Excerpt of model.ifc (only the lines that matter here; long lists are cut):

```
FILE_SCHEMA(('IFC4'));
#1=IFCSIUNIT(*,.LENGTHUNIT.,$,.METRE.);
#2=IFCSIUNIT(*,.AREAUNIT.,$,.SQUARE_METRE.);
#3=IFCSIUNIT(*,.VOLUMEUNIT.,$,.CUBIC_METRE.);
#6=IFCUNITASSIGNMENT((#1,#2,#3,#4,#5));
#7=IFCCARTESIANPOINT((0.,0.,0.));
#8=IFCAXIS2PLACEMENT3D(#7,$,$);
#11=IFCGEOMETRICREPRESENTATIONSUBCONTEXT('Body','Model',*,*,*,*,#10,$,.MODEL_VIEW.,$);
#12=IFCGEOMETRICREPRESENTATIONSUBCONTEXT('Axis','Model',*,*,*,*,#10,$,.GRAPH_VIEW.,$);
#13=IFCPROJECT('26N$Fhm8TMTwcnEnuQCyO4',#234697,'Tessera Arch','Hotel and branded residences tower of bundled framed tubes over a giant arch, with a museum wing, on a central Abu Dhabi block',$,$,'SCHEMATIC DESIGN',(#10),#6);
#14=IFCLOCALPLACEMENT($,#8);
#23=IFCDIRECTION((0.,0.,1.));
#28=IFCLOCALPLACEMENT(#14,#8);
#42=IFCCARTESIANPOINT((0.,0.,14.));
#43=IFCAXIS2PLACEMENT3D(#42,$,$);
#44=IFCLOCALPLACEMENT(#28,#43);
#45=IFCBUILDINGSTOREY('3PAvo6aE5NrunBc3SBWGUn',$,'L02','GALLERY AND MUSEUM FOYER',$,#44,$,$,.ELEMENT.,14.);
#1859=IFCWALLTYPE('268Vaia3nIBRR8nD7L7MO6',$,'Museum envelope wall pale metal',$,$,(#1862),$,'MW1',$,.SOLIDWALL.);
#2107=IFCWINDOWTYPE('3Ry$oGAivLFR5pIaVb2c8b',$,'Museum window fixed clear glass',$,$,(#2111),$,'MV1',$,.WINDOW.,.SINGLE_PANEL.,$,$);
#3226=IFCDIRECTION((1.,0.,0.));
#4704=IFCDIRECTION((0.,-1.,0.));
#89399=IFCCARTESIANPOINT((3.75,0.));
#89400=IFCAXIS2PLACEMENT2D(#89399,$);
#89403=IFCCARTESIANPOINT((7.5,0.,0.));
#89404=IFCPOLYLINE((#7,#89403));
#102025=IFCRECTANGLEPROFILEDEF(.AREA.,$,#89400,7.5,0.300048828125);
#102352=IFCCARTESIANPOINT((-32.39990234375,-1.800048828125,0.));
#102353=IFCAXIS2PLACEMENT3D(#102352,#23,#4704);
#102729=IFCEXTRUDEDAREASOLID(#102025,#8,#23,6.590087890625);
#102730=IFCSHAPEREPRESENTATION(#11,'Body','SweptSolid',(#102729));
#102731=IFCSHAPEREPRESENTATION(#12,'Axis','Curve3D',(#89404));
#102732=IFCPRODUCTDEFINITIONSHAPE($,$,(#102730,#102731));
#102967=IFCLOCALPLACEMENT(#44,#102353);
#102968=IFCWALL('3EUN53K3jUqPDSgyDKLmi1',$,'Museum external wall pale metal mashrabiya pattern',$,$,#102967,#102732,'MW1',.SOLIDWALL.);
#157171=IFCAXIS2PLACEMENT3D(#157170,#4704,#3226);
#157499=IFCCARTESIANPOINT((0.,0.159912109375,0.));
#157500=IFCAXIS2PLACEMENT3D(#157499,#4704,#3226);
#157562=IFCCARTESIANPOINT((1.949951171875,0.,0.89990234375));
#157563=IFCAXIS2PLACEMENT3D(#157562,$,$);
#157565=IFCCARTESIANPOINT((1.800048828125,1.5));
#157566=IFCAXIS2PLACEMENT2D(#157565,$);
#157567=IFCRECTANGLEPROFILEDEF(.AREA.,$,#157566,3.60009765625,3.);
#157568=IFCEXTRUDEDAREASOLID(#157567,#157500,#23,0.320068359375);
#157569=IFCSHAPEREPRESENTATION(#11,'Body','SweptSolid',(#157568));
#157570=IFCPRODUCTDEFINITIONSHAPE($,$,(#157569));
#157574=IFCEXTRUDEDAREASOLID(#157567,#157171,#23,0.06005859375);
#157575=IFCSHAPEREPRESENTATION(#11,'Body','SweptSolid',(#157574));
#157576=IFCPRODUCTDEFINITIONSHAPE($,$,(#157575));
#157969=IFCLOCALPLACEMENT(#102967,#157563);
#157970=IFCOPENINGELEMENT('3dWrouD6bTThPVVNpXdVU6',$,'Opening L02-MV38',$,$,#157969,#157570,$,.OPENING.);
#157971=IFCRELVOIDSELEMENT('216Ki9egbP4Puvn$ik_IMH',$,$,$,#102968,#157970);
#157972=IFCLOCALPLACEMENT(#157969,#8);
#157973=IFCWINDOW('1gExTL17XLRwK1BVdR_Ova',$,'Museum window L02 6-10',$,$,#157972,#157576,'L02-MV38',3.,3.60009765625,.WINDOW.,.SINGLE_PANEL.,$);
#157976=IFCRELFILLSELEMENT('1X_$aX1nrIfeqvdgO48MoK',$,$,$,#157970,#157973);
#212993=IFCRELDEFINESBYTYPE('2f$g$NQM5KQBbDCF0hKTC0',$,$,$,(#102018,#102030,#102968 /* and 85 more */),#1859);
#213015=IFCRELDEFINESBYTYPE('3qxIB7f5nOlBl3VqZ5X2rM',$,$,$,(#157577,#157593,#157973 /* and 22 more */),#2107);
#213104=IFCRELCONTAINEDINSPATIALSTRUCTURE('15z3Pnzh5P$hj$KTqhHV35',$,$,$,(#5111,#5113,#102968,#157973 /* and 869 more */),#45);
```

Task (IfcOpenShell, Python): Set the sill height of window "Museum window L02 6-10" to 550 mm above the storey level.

```python
import numpy as np
import ifcopenshell
import ifcopenshell.api.geometry
import ifcopenshell.geom
import ifcopenshell.util.element
import ifcopenshell.util.placement
import ifcopenshell.util.shape
import ifcopenshell.util.unit

model = ifcopenshell.open("model.ifc")
unit_scale = ifcopenshell.util.unit.calculate_unit_scale(model)

window = model.by_guid("1gExTL17XLRwK1BVdR_Ova")
opening = window.FillsVoids[0].RelatingOpeningElement
storey = ifcopenshell.util.element.get_container(window, ifc_class="IfcBuildingStorey")
level = ifcopenshell.util.placement.get_local_placement(storey.ObjectPlacement)[2, 3]

# The opening's origin need not be at the sill, so measure its lowest point.
shape = ifcopenshell.geom.create_shape(ifcopenshell.geom.settings(), opening)
bottom = ifcopenshell.util.shape.get_shape_bottom_elevation(shape, shape.geometry) / unit_scale
dz = level + 0.55 - bottom

shift = np.array([0.0, 0.0, dz])
# The window is placed relative to its opening, so it follows when the opening moves.
matrix = ifcopenshell.util.placement.get_local_placement(opening.ObjectPlacement)
matrix[:3, 3] += shift
ifcopenshell.api.geometry.edit_object_placement(
    model, product=opening, matrix=matrix, is_si=False, should_transform_children=True
)

print(f"moved by {dz * unit_scale:+.3f} m")

model.write("model_edited.ifc")
```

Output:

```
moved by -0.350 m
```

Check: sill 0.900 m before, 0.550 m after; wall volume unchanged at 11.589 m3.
